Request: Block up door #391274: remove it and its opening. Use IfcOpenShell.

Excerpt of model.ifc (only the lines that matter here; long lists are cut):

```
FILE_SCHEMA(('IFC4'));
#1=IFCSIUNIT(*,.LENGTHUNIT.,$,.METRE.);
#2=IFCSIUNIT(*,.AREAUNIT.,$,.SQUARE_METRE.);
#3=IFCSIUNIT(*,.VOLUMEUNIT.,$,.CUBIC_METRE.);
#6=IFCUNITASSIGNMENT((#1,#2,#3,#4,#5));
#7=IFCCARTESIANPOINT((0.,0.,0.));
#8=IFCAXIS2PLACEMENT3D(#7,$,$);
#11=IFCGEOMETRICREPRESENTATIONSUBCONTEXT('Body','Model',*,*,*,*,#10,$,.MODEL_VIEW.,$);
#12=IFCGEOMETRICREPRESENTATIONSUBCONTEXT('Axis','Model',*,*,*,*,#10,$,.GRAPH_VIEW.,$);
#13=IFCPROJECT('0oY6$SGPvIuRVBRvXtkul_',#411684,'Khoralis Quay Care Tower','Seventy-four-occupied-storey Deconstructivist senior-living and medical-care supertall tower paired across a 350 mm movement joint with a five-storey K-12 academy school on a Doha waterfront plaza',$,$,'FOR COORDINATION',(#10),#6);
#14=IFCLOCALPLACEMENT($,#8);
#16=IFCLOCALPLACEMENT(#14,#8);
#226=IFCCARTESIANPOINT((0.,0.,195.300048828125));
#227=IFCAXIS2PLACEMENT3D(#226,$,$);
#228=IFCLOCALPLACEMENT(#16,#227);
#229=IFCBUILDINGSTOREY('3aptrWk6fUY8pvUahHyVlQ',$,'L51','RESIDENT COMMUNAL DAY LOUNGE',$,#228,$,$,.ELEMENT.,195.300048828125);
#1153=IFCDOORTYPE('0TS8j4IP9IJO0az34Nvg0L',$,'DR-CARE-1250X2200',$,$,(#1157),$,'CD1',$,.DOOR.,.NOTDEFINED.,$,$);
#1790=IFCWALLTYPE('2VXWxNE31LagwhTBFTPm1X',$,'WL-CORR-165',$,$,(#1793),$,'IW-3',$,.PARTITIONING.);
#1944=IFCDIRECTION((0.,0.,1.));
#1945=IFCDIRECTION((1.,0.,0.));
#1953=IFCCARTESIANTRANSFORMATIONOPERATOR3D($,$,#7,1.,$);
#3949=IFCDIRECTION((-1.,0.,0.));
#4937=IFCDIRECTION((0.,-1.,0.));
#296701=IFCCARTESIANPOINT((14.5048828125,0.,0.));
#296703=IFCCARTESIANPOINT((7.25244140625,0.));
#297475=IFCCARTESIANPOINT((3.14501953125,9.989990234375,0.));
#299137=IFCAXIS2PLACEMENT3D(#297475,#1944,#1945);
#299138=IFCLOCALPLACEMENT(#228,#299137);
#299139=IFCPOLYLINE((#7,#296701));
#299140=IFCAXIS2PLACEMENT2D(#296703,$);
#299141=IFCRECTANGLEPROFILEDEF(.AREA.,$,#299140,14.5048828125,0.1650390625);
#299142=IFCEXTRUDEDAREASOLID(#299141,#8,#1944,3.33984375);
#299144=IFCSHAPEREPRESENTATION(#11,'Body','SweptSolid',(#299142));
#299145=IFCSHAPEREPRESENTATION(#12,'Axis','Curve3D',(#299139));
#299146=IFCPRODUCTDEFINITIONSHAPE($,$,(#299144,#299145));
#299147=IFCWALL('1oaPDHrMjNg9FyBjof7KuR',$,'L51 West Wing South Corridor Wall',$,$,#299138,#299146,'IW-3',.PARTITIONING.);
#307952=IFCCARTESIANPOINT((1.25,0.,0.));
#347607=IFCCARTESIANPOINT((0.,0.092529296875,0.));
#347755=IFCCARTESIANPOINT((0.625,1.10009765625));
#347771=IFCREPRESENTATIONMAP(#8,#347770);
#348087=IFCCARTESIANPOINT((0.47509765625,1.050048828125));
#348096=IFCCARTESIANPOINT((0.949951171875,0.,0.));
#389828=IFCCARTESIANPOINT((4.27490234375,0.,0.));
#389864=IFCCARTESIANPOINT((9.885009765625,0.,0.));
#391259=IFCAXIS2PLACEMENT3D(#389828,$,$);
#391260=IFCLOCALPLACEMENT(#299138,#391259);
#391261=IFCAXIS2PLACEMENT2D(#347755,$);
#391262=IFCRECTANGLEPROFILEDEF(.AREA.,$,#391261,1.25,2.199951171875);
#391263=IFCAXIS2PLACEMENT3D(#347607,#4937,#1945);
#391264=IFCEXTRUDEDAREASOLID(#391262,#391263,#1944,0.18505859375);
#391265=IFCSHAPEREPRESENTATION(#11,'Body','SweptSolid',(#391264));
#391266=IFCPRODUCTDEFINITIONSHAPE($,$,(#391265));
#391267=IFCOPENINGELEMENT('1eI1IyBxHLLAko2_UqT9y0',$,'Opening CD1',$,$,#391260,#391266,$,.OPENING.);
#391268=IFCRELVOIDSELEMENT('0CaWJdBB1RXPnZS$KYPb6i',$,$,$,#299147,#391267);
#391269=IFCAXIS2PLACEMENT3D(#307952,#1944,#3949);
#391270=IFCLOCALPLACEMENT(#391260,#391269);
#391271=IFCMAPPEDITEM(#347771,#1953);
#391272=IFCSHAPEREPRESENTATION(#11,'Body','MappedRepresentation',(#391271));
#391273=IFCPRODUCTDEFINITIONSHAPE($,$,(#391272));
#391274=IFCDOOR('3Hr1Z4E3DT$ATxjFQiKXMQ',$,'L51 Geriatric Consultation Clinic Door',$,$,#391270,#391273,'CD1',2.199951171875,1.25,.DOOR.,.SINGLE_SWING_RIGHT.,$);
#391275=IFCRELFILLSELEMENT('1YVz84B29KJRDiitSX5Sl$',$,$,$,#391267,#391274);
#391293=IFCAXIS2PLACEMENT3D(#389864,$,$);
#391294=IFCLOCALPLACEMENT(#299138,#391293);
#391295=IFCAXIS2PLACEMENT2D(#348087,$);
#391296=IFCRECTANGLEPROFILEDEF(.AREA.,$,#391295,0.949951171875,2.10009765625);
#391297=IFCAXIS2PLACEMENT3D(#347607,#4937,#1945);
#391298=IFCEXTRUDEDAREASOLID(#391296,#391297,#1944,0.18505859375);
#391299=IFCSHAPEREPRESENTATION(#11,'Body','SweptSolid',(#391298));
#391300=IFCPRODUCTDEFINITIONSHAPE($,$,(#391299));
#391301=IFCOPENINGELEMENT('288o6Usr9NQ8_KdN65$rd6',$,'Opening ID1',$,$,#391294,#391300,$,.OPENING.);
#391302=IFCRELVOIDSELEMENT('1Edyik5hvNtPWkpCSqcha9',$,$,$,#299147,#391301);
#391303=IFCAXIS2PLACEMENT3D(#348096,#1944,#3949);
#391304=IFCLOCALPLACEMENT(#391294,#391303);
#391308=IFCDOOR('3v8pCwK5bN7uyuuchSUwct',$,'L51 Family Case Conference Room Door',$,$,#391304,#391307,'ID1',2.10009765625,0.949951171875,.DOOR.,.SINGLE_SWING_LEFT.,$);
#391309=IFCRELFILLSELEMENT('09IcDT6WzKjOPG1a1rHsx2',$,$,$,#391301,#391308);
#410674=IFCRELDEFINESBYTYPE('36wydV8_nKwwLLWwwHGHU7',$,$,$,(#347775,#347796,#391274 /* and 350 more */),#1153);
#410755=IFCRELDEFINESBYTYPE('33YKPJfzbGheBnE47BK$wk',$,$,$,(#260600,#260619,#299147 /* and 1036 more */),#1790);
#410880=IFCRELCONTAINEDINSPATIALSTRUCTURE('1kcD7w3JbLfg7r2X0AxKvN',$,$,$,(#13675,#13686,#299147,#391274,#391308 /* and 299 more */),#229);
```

```python
import ifcopenshell
import ifcopenshell.api.feature
import ifcopenshell.api.root
import ifcopenshell.geom
import ifcopenshell.util.shape

model = ifcopenshell.open("model.ifc")
settings = ifcopenshell.geom.settings()


def volume(element):
    """Net volume in cubic metres, openings subtracted."""
    shape = ifcopenshell.geom.create_shape(settings, element)
    return ifcopenshell.util.shape.get_volume(shape.geometry)


door = model.by_guid("3Hr1Z4E3DT$ATxjFQiKXMQ")
opening = door.FillsVoids[0].RelatingOpeningElement
wall = opening.VoidsElements[0].RelatingBuildingElement
before = volume(wall)

ifcopenshell.api.root.remove_product(model, product=door)
ifcopenshell.api.feature.remove_feature(model, feature=opening)

after = volume(wall)

print(f"wall volume {before:.3f} -> {after:.3f} m3")

model.write("model-out.ifc")
```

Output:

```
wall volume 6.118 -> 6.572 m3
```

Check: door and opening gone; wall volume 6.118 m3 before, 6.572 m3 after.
